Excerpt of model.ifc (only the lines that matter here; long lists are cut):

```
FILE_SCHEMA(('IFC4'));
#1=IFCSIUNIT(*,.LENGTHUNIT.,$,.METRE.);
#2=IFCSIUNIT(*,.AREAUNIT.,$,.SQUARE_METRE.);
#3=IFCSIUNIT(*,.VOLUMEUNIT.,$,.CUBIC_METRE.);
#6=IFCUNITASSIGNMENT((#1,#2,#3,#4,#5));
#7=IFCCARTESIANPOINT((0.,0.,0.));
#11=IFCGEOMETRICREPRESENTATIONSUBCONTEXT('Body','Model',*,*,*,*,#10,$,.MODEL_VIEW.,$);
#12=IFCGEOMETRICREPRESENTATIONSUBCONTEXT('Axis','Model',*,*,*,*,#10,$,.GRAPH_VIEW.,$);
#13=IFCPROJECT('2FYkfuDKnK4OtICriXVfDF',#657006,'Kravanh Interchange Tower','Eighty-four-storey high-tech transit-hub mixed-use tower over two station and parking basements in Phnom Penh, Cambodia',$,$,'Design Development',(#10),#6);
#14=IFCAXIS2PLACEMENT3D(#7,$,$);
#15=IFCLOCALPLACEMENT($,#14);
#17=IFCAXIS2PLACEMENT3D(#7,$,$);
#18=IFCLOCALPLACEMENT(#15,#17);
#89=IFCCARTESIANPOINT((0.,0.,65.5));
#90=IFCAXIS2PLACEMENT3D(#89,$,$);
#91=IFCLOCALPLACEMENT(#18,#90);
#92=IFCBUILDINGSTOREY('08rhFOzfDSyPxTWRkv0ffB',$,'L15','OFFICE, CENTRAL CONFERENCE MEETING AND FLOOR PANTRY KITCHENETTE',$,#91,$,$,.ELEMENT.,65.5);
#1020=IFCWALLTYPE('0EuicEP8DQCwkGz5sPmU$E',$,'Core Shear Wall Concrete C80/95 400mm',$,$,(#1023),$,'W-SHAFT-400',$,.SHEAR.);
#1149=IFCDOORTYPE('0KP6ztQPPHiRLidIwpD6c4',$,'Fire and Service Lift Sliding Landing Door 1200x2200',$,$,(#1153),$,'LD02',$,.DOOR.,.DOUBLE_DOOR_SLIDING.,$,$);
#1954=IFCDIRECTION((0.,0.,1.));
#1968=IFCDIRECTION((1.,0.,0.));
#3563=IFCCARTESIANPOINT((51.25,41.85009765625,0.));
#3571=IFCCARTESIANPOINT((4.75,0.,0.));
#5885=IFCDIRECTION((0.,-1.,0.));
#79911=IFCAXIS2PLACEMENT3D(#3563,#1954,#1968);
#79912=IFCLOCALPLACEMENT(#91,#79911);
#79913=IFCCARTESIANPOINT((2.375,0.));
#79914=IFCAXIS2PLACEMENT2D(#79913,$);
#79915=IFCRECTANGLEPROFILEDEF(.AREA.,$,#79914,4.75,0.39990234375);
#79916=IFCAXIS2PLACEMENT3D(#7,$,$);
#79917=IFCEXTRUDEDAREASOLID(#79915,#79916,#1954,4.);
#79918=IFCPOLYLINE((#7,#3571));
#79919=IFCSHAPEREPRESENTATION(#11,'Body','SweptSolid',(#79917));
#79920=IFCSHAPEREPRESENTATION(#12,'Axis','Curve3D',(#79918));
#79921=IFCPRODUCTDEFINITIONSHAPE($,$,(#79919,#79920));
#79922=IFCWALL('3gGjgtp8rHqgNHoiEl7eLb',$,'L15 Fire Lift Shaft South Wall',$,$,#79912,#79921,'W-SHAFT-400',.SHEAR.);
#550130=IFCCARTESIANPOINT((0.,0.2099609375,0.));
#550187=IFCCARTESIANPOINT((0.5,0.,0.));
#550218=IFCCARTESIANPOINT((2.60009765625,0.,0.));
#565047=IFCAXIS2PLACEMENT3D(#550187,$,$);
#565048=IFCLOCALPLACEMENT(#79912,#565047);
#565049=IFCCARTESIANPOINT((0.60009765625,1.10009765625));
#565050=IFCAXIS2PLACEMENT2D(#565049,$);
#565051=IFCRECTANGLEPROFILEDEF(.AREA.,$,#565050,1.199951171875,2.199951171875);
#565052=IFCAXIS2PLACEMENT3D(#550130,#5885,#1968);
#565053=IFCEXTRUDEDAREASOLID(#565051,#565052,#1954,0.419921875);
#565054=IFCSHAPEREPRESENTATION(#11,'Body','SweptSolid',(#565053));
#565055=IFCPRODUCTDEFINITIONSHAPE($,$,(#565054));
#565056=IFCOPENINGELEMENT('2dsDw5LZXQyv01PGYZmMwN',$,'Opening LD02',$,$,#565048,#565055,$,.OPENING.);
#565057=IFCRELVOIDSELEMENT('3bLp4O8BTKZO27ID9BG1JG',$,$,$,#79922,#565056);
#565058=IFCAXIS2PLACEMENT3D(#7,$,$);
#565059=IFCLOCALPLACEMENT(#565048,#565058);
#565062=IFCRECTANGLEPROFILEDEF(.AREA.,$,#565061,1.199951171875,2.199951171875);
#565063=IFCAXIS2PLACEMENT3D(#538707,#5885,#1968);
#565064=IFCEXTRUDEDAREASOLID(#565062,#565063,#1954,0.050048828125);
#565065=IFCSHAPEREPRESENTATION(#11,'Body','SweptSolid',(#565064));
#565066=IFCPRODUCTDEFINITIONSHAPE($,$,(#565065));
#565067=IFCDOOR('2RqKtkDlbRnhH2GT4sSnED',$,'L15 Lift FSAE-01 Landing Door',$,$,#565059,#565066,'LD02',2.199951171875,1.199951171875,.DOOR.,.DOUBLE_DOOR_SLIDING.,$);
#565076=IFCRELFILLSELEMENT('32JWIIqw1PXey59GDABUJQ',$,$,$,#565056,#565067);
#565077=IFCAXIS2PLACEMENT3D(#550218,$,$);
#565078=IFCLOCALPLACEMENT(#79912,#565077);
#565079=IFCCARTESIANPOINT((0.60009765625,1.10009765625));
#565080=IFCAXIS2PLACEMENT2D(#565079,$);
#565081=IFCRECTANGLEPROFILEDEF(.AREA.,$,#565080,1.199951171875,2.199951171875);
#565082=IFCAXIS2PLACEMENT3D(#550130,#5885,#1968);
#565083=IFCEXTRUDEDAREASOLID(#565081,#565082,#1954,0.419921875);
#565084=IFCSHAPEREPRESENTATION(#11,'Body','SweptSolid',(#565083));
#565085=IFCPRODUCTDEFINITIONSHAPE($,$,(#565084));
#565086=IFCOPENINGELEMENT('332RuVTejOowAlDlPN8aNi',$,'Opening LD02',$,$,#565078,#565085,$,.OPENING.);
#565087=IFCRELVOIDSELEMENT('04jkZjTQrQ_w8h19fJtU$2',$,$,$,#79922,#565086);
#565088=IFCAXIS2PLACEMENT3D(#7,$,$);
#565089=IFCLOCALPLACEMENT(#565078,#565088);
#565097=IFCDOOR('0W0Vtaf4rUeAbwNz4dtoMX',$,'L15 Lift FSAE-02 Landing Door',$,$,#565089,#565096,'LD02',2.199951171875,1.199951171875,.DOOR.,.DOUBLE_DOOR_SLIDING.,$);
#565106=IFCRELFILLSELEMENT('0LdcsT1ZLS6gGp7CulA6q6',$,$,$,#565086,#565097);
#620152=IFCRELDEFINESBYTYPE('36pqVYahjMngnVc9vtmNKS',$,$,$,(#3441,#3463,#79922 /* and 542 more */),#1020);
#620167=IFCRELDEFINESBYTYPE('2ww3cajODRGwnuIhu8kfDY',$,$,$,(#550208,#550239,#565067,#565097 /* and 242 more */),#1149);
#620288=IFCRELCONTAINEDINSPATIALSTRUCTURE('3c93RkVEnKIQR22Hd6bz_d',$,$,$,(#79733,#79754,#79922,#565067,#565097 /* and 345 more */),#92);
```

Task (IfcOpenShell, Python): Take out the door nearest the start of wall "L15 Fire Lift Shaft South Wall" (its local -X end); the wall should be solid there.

```python
import ifcopenshell
import ifcopenshell.api.feature
import ifcopenshell.api.root
import ifcopenshell.geom
import ifcopenshell.util.shape

model = ifcopenshell.open("model.ifc")
settings = ifcopenshell.geom.settings()


def volume(element):
    """Net volume in cubic metres, openings subtracted."""
    shape = ifcopenshell.geom.create_shape(settings, element)
    return ifcopenshell.util.shape.get_volume(shape.geometry)


door = model.by_id(565067)
opening = door.FillsVoids[0].RelatingOpeningElement
wall = opening.VoidsElements[0].RelatingBuildingElement
before = volume(wall)

ifcopenshell.api.root.remove_product(model, product=door)
ifcopenshell.api.feature.remove_feature(model, feature=opening)

after = volume(wall)

print(f"wall volume {before:.3f} -> {after:.3f} m3")

model.write("model_edited.ifc")
```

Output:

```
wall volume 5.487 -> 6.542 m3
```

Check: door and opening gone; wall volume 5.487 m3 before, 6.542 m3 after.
